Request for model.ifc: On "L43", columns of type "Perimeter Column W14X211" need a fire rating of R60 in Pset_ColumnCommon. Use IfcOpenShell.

First a look at what the model holds.

```python
import ifcopenshell
import ifcopenshell.util.element

model = ifcopenshell.open("model.ifc")
print(model.schema)
storey = next(s for s in model.by_type("IfcBuildingStorey") if s.Name == "L43")
columns = [e for e in ifcopenshell.util.element.get_decomposition(storey) if e.is_a("IfcColumn")]
seen = {}
for e in columns:
    element_type = ifcopenshell.util.element.get_type(e)
    key = (element_type.Name if element_type != e and element_type else None, ifcopenshell.util.element.get_pset(e, "Pset_ColumnCommon", "FireRating"))
    seen[key] = seen.get(key, 0) + 1
for (name, value), count in sorted(seen.items(), key=str):
    print(count, "x", name, "|", value)
```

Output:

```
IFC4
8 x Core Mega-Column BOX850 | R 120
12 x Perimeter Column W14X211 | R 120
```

```python
import ifcopenshell
import ifcopenshell.api.pset
import ifcopenshell.util.element

model = ifcopenshell.open("model.ifc")

storey = next(s for s in model.by_type("IfcBuildingStorey") if s.Name == "L43")
columns = [e for e in ifcopenshell.util.element.get_decomposition(storey) if e.is_a("IfcColumn")]

count = 0
for e in columns:
    element_type = ifcopenshell.util.element.get_type(e)
    if element_type in (None, e) or element_type.Name != "Perimeter Column W14X211":
        continue
    found = ifcopenshell.util.element.get_pset(e, "Pset_ColumnCommon", should_inherit=False)
    if found:
        pset = model.by_id(found["id"])
        if len(ifcopenshell.util.element.get_elements_by_pset(pset)) > 1:
            pset = ifcopenshell.api.pset.unshare_pset(model, products=[e], pset=pset)[0]
    else:
        pset = ifcopenshell.api.pset.add_pset(model, product=e, name="Pset_ColumnCommon")
    ifcopenshell.api.pset.edit_pset(model, pset=pset, properties={"FireRating": "R60"})
    count += 1

print(count, "columns updated")

model.write("model_v2.ifc")
```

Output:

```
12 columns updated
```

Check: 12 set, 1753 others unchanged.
